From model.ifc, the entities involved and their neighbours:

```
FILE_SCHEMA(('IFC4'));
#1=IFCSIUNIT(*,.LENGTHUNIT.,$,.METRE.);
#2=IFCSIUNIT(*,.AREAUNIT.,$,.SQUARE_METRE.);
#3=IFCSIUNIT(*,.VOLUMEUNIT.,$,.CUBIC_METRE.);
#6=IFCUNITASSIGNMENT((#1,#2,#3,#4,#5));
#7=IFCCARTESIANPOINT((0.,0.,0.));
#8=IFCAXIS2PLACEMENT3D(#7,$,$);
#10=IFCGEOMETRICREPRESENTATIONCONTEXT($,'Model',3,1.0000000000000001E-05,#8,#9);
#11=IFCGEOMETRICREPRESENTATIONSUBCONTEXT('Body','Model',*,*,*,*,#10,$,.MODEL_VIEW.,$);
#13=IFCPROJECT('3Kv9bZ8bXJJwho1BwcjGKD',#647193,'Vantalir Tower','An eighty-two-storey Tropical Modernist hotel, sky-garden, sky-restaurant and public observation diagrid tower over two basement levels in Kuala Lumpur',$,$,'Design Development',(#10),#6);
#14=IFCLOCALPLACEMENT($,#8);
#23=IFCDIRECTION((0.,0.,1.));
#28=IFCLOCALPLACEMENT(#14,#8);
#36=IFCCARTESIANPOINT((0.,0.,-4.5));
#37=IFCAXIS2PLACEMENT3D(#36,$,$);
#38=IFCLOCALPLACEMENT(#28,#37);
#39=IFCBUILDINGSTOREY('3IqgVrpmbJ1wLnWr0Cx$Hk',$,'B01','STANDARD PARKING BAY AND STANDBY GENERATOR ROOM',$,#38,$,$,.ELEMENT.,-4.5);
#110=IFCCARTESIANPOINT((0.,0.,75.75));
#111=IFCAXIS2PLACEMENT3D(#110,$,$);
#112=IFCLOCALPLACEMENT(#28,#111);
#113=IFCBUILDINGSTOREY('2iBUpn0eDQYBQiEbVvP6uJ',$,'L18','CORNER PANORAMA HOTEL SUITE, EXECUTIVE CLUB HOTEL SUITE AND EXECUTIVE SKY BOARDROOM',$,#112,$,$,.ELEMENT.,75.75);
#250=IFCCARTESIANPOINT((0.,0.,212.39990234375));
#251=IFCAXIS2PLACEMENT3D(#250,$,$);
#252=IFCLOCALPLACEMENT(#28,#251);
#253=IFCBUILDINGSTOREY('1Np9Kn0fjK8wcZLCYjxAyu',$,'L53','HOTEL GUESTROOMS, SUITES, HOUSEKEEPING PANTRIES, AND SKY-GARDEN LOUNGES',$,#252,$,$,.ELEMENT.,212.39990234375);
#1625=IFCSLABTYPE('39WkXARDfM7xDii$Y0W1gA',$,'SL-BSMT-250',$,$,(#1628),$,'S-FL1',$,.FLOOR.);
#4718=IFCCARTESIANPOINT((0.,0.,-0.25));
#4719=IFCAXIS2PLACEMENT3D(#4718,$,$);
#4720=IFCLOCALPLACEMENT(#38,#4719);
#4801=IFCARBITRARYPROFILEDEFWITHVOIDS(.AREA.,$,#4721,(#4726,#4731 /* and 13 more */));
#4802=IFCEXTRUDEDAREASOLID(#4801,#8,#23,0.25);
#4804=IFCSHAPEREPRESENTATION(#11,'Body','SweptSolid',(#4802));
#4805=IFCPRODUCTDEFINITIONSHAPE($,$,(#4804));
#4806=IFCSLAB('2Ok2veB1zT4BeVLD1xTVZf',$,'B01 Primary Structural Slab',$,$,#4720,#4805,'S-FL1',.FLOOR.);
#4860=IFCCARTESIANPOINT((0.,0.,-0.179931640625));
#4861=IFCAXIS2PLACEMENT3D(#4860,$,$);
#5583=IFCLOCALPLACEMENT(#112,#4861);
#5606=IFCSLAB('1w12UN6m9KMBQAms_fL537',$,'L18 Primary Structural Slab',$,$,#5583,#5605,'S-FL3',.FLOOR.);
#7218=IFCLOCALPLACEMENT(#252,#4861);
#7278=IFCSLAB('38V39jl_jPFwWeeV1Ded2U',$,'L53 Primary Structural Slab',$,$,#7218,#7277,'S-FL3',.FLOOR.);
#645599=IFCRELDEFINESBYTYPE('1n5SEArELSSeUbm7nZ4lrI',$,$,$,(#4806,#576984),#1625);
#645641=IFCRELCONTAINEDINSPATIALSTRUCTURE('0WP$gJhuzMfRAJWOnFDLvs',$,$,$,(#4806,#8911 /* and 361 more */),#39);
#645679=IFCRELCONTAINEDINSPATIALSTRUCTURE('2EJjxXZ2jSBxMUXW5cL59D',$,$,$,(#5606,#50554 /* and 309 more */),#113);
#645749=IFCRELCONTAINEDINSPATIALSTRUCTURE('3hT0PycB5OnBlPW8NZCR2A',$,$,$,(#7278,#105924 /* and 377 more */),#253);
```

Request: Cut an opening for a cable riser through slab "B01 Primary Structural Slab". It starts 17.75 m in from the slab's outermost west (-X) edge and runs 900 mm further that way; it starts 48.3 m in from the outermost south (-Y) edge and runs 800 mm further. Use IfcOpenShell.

```python
import numpy as np
import ifcopenshell
import ifcopenshell.api.feature
import ifcopenshell.api.geometry
import ifcopenshell.api.root
import ifcopenshell.geom
import ifcopenshell.util.placement
import ifcopenshell.util.representation
import ifcopenshell.util.shape
import ifcopenshell.util.unit

model = ifcopenshell.open("model.ifc")
unit_scale = ifcopenshell.util.unit.calculate_unit_scale(model)
settings = ifcopenshell.geom.settings()


def volume(element):
    """Net volume in cubic metres, openings subtracted."""
    shape = ifcopenshell.geom.create_shape(settings, element)
    return ifcopenshell.util.shape.get_volume(shape.geometry)


slab = model.by_guid("2Ok2veB1zT4BeVLD1xTVZf")
before = volume(slab)

# Extent in the slab's own axes, in metres. The edges named are its -X and -Y sides.
slab_shape = ifcopenshell.geom.create_shape(settings, slab)
vertices = ifcopenshell.util.shape.get_vertices(slab_shape.geometry)
x_min, y_min, bottom = vertices.min(axis=0)
top = vertices[:, 2].max()

opening = ifcopenshell.api.root.create_entity(model, ifc_class="IfcOpeningElement", name="Cable riser opening", predefined_type="OPENING")
context = ifcopenshell.util.representation.get_context(model, "Model", "Body", "MODEL_VIEW")
width, depth = 0.9, 0.8
outline = [(0.0, 0.0), (width, 0.0), (width, depth), (0.0, depth), (0.0, 0.0)]
# Overshoot both faces by 50 mm so the cut is clean.
shape = ifcopenshell.api.geometry.add_slab_representation(
    model, context=context, depth=top - bottom + 0.1, polyline=outline
)
ifcopenshell.api.geometry.assign_representation(model, product=opening, representation=shape)

matrix = ifcopenshell.util.placement.get_local_placement(slab.ObjectPlacement)
matrix[:, 3] = matrix @ np.append(np.array([x_min + 17.75, y_min + 48.3, bottom - 0.05]) / unit_scale, 1.0)
ifcopenshell.api.geometry.edit_object_placement(model, product=opening, matrix=matrix, is_si=False)
ifcopenshell.api.feature.add_feature(model, feature=opening, element=slab)

after = volume(slab)

print(f"slab volume {before:.3f} -> {after:.3f} m3")

model.write("model_v2.ifc")
```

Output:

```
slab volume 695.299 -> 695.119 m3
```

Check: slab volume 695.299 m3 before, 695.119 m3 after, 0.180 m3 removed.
